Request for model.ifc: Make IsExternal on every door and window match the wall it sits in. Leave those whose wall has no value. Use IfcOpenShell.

First a look at what the model holds.

```python
import ifcopenshell
import ifcopenshell.util.element

model = ifcopenshell.open("model.ifc")
print(model.schema)
seen = {}
for e in model.by_type("IfcDoor") + model.by_type("IfcWindow"):
    if not e.FillsVoids:
        continue
    host = e.FillsVoids[0].RelatingOpeningElement.VoidsElements[0].RelatingBuildingElement
    own = ifcopenshell.util.element.get_pset(e, f"Pset_{e.is_a()[3:].removesuffix('StandardCase')}Common", "IsExternal")
    wall = ifcopenshell.util.element.get_pset(host, "Pset_WallCommon", "IsExternal")
    seen[e.is_a(), own, wall] = seen.get((e.is_a(), own, wall), 0) + 1
for (cls, own, wall), count in sorted(seen.items(), key=str):
    print(count, cls, "IsExternal:", own, "| host wall:", wall)
```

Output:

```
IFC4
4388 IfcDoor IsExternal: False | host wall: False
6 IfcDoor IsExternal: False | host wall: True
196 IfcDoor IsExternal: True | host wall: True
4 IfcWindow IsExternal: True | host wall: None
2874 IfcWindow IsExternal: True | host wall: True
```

```python
import ifcopenshell
import ifcopenshell.api.pset
import ifcopenshell.util.element

model = ifcopenshell.open("model.ifc")

count = 0
for ifc_class, pset_name in (("IfcDoor", "Pset_DoorCommon"), ("IfcWindow", "Pset_WindowCommon")):
    for e in model.by_type(ifc_class):
        if not e.FillsVoids:
            continue
        host = e.FillsVoids[0].RelatingOpeningElement.VoidsElements[0].RelatingBuildingElement
        external = ifcopenshell.util.element.get_pset(host, "Pset_WallCommon", "IsExternal")
        if external is None or ifcopenshell.util.element.get_pset(e, pset_name, "IsExternal") == external:
            continue
        pset = ifcopenshell.api.pset.add_pset(model, product=e, name=pset_name)
        ifcopenshell.api.pset.edit_pset(model, pset=pset, properties={"IsExternal": external})
        count += 1

print(count, "updated")

model.write("model_updated.ifc")
```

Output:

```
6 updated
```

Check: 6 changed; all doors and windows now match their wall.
